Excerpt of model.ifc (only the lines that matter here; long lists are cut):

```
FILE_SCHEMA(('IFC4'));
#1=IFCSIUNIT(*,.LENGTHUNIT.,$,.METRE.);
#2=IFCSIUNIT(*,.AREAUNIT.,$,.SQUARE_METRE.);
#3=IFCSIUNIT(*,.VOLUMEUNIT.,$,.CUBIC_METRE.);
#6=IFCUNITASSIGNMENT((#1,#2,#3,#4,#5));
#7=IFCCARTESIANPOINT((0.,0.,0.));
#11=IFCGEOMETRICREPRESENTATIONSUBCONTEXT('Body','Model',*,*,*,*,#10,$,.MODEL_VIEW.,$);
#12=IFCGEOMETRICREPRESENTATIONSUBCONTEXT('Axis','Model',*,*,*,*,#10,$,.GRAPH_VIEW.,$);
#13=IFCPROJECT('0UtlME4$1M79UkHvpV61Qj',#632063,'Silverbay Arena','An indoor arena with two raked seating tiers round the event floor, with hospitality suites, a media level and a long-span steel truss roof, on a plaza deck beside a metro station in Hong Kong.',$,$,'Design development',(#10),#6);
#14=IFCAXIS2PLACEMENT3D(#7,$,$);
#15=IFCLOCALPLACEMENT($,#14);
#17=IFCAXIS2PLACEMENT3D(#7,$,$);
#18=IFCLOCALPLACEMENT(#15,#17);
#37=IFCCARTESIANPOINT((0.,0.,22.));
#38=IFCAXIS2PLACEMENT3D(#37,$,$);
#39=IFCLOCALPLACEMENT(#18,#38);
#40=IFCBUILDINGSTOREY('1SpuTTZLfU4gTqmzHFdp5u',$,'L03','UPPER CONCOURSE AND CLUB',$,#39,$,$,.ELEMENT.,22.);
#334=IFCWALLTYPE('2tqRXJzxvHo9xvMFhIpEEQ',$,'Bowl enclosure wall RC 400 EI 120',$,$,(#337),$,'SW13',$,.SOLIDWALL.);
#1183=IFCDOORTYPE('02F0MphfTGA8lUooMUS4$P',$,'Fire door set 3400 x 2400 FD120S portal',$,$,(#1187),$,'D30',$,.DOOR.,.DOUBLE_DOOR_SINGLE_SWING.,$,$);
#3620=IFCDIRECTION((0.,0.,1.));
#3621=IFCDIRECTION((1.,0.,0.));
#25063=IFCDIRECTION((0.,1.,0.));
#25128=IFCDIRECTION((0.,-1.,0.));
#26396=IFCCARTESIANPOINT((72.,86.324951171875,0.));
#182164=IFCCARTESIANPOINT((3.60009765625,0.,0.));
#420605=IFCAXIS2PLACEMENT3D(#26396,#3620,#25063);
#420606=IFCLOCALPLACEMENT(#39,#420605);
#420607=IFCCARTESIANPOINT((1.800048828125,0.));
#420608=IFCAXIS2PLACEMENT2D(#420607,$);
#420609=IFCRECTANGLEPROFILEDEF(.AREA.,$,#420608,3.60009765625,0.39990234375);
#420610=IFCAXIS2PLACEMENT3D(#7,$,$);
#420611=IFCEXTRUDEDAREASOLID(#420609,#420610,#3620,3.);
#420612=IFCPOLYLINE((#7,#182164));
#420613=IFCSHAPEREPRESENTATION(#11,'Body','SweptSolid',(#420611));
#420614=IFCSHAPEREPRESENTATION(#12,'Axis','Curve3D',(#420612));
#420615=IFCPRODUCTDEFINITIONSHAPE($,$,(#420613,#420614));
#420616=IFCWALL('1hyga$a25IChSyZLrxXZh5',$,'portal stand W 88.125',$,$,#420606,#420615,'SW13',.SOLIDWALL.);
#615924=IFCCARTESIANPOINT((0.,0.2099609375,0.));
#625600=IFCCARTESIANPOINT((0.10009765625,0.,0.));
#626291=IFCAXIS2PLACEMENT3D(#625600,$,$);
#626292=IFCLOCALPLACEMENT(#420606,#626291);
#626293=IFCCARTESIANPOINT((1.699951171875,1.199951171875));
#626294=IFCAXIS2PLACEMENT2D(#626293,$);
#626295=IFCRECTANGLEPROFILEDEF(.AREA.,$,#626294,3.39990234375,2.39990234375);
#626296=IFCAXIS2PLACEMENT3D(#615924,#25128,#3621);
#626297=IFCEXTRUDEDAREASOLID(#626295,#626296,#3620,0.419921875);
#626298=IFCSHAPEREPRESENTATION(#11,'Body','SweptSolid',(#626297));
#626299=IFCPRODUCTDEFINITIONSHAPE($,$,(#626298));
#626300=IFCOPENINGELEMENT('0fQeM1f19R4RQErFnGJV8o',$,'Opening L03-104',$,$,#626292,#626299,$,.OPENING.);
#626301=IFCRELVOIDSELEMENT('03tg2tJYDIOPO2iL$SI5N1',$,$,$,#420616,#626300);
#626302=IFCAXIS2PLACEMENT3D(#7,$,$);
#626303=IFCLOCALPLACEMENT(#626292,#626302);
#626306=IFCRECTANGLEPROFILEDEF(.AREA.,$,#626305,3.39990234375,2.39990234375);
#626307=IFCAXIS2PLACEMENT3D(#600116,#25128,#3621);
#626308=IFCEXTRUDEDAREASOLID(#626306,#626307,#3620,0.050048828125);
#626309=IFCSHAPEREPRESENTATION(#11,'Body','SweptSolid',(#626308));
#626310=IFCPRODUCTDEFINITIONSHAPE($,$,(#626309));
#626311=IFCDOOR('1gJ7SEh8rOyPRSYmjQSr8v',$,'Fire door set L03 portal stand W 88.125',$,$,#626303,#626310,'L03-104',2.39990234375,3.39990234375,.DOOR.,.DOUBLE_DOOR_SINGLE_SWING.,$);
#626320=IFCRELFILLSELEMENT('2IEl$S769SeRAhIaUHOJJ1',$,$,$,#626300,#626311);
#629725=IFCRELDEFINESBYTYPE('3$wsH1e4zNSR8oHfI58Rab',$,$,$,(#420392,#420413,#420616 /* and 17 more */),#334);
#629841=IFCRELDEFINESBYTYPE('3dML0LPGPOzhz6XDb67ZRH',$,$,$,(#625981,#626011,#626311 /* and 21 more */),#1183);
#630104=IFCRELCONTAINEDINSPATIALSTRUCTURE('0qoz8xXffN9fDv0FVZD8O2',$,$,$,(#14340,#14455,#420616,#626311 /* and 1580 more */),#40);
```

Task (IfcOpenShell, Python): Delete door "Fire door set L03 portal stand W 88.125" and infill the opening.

```python
import ifcopenshell
import ifcopenshell.api.feature
import ifcopenshell.api.root
import ifcopenshell.geom
import ifcopenshell.util.shape

model = ifcopenshell.open("model.ifc")
settings = ifcopenshell.geom.settings()


def volume(element):
    """Net volume in cubic metres, openings subtracted."""
    shape = ifcopenshell.geom.create_shape(settings, element)
    return ifcopenshell.util.shape.get_volume(shape.geometry)


door = model.by_id(626311)
opening = door.FillsVoids[0].RelatingOpeningElement
wall = opening.VoidsElements[0].RelatingBuildingElement
before = volume(wall)

ifcopenshell.api.root.remove_product(model, product=door)
ifcopenshell.api.feature.remove_feature(model, feature=opening)

after = volume(wall)

print(f"wall volume {before:.3f} -> {after:.3f} m3")

model.write("model-out.ifc")
```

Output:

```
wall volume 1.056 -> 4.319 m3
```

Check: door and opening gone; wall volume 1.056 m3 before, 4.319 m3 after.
